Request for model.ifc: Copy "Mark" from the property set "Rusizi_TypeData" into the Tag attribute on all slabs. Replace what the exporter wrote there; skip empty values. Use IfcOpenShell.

First a look at what the model holds.

```python
import ifcopenshell
import ifcopenshell.util.element

model = ifcopenshell.open("model.ifc")
print(model.schema)
slabs = model.by_type("IfcSlab")
print(len(slabs), "slabs")
for e in slabs[:8]:
    source = ifcopenshell.util.element.get_pset(e, "Rusizi_TypeData", "Mark")
    target = e.Tag
    print(e.id(), repr(source), repr(target), sep=" | ")
```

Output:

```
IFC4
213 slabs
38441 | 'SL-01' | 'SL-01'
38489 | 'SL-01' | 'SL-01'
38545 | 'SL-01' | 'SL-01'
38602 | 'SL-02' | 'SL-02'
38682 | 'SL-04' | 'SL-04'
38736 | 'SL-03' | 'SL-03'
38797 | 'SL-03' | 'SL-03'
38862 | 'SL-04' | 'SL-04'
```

```python
import ifcopenshell
import ifcopenshell.util.element

model = ifcopenshell.open("model.ifc")

count = 0
for e in model.by_type("IfcSlab"):
    value = ifcopenshell.util.element.get_pset(e, "Rusizi_TypeData", "Mark")
    current = e.Tag
    if not value or not value.strip() or current == value:
        continue
    e.Tag = value
    count += 1

print(count, "slabs updated")

model.write("model_updated.ifc")
```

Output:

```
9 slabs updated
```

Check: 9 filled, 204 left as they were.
